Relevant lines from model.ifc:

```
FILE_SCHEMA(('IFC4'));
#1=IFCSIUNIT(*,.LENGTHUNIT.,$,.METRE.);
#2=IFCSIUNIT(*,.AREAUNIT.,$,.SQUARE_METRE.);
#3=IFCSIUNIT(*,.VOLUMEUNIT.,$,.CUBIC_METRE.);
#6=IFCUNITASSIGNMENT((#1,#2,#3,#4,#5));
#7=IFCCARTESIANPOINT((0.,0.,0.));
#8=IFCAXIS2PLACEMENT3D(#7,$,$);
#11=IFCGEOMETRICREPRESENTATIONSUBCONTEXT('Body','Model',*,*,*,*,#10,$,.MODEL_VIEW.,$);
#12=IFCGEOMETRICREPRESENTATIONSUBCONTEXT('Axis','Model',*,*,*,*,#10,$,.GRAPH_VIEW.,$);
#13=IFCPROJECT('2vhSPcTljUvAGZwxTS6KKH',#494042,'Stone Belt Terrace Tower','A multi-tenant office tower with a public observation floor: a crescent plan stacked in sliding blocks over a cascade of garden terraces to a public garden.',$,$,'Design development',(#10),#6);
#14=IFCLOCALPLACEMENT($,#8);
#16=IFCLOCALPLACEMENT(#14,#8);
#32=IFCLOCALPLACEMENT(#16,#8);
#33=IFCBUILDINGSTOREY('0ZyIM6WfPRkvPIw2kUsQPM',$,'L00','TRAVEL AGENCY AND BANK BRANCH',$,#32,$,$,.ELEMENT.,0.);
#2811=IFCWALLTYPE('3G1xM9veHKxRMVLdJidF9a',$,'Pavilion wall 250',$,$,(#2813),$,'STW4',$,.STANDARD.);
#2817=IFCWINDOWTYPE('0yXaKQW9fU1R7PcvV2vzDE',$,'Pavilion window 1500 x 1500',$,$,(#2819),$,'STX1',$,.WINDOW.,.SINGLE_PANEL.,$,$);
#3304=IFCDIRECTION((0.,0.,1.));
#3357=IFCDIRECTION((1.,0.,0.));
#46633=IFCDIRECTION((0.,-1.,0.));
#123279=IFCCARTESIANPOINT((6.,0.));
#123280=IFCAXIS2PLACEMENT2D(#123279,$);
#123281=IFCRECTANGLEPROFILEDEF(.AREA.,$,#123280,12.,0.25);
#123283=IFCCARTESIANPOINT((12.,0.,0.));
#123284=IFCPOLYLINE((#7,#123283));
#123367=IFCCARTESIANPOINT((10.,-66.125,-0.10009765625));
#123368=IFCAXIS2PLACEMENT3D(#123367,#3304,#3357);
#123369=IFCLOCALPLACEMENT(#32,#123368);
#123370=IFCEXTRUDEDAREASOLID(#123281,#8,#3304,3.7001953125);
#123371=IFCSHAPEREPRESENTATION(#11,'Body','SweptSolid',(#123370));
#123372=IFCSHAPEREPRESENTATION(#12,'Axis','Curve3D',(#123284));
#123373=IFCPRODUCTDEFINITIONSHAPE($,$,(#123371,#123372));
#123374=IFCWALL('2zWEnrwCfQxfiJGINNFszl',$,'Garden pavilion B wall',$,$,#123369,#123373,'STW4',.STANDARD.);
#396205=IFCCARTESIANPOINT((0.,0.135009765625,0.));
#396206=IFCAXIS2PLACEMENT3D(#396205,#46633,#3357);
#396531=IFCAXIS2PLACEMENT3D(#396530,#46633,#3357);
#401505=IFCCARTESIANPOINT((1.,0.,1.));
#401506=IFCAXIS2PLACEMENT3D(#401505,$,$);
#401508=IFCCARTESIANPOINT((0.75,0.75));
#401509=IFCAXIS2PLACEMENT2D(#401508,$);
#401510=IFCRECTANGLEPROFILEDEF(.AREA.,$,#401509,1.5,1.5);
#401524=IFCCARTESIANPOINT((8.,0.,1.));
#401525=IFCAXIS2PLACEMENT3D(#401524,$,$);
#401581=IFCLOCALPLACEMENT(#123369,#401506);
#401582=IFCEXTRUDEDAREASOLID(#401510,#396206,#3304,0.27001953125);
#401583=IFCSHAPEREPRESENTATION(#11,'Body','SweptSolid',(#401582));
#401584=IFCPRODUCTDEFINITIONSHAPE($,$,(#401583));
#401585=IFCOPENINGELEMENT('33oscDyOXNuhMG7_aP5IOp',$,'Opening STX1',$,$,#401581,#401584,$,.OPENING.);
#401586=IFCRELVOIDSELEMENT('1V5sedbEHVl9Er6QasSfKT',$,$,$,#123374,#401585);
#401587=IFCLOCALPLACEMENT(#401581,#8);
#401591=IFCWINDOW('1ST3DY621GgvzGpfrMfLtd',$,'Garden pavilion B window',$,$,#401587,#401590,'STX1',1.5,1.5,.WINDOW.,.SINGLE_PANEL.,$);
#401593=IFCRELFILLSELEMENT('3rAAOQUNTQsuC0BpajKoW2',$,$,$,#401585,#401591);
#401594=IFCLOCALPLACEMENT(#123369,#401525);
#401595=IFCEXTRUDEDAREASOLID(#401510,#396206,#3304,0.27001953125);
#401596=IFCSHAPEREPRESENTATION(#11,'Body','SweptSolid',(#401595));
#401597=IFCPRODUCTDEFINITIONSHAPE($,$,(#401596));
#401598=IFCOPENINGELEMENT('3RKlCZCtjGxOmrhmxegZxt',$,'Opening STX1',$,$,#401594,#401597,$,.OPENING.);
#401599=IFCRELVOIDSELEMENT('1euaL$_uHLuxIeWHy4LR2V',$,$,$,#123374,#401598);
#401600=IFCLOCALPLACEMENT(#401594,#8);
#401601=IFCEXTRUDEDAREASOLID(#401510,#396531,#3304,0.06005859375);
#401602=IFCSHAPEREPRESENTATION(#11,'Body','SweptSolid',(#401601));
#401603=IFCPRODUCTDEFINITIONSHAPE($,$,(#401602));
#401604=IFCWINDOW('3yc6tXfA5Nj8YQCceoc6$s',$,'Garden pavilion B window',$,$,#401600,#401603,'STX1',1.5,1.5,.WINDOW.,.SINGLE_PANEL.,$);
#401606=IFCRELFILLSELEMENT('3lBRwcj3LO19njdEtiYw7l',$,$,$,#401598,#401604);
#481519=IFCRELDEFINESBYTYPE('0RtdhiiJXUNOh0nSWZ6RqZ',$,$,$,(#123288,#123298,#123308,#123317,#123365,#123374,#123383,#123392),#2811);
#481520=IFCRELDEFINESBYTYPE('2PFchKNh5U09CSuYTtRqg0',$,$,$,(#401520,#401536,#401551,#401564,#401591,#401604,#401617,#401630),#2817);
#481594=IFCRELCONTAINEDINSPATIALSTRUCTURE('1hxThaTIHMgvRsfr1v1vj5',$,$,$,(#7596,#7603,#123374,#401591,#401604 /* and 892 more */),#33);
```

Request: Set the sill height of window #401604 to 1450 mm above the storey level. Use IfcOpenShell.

```python
import numpy as np
import ifcopenshell
import ifcopenshell.api.geometry
import ifcopenshell.geom
import ifcopenshell.util.element
import ifcopenshell.util.placement
import ifcopenshell.util.shape
import ifcopenshell.util.unit

model = ifcopenshell.open("model.ifc")
unit_scale = ifcopenshell.util.unit.calculate_unit_scale(model)

window = model.by_guid("3yc6tXfA5Nj8YQCceoc6$s")
opening = window.FillsVoids[0].RelatingOpeningElement
storey = ifcopenshell.util.element.get_container(window, ifc_class="IfcBuildingStorey")
level = ifcopenshell.util.placement.get_local_placement(storey.ObjectPlacement)[2, 3]

# The opening's origin need not be at the sill, so measure its lowest point.
shape = ifcopenshell.geom.create_shape(ifcopenshell.geom.settings(), opening)
bottom = ifcopenshell.util.shape.get_shape_bottom_elevation(shape, shape.geometry) / unit_scale
dz = level + 1.45 / unit_scale - bottom

shift = np.array([0.0, 0.0, dz])
# The window is placed relative to its opening, so it follows when the opening moves.
matrix = ifcopenshell.util.placement.get_local_placement(opening.ObjectPlacement)
matrix[:3, 3] += shift
ifcopenshell.api.geometry.edit_object_placement(
    model, product=opening, matrix=matrix, is_si=False, should_transform_children=True
)

print(f"moved by {dz * unit_scale:+.3f} m")

model.write("model_v2.ifc")
```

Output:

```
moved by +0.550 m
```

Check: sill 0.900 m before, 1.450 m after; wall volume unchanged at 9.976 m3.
